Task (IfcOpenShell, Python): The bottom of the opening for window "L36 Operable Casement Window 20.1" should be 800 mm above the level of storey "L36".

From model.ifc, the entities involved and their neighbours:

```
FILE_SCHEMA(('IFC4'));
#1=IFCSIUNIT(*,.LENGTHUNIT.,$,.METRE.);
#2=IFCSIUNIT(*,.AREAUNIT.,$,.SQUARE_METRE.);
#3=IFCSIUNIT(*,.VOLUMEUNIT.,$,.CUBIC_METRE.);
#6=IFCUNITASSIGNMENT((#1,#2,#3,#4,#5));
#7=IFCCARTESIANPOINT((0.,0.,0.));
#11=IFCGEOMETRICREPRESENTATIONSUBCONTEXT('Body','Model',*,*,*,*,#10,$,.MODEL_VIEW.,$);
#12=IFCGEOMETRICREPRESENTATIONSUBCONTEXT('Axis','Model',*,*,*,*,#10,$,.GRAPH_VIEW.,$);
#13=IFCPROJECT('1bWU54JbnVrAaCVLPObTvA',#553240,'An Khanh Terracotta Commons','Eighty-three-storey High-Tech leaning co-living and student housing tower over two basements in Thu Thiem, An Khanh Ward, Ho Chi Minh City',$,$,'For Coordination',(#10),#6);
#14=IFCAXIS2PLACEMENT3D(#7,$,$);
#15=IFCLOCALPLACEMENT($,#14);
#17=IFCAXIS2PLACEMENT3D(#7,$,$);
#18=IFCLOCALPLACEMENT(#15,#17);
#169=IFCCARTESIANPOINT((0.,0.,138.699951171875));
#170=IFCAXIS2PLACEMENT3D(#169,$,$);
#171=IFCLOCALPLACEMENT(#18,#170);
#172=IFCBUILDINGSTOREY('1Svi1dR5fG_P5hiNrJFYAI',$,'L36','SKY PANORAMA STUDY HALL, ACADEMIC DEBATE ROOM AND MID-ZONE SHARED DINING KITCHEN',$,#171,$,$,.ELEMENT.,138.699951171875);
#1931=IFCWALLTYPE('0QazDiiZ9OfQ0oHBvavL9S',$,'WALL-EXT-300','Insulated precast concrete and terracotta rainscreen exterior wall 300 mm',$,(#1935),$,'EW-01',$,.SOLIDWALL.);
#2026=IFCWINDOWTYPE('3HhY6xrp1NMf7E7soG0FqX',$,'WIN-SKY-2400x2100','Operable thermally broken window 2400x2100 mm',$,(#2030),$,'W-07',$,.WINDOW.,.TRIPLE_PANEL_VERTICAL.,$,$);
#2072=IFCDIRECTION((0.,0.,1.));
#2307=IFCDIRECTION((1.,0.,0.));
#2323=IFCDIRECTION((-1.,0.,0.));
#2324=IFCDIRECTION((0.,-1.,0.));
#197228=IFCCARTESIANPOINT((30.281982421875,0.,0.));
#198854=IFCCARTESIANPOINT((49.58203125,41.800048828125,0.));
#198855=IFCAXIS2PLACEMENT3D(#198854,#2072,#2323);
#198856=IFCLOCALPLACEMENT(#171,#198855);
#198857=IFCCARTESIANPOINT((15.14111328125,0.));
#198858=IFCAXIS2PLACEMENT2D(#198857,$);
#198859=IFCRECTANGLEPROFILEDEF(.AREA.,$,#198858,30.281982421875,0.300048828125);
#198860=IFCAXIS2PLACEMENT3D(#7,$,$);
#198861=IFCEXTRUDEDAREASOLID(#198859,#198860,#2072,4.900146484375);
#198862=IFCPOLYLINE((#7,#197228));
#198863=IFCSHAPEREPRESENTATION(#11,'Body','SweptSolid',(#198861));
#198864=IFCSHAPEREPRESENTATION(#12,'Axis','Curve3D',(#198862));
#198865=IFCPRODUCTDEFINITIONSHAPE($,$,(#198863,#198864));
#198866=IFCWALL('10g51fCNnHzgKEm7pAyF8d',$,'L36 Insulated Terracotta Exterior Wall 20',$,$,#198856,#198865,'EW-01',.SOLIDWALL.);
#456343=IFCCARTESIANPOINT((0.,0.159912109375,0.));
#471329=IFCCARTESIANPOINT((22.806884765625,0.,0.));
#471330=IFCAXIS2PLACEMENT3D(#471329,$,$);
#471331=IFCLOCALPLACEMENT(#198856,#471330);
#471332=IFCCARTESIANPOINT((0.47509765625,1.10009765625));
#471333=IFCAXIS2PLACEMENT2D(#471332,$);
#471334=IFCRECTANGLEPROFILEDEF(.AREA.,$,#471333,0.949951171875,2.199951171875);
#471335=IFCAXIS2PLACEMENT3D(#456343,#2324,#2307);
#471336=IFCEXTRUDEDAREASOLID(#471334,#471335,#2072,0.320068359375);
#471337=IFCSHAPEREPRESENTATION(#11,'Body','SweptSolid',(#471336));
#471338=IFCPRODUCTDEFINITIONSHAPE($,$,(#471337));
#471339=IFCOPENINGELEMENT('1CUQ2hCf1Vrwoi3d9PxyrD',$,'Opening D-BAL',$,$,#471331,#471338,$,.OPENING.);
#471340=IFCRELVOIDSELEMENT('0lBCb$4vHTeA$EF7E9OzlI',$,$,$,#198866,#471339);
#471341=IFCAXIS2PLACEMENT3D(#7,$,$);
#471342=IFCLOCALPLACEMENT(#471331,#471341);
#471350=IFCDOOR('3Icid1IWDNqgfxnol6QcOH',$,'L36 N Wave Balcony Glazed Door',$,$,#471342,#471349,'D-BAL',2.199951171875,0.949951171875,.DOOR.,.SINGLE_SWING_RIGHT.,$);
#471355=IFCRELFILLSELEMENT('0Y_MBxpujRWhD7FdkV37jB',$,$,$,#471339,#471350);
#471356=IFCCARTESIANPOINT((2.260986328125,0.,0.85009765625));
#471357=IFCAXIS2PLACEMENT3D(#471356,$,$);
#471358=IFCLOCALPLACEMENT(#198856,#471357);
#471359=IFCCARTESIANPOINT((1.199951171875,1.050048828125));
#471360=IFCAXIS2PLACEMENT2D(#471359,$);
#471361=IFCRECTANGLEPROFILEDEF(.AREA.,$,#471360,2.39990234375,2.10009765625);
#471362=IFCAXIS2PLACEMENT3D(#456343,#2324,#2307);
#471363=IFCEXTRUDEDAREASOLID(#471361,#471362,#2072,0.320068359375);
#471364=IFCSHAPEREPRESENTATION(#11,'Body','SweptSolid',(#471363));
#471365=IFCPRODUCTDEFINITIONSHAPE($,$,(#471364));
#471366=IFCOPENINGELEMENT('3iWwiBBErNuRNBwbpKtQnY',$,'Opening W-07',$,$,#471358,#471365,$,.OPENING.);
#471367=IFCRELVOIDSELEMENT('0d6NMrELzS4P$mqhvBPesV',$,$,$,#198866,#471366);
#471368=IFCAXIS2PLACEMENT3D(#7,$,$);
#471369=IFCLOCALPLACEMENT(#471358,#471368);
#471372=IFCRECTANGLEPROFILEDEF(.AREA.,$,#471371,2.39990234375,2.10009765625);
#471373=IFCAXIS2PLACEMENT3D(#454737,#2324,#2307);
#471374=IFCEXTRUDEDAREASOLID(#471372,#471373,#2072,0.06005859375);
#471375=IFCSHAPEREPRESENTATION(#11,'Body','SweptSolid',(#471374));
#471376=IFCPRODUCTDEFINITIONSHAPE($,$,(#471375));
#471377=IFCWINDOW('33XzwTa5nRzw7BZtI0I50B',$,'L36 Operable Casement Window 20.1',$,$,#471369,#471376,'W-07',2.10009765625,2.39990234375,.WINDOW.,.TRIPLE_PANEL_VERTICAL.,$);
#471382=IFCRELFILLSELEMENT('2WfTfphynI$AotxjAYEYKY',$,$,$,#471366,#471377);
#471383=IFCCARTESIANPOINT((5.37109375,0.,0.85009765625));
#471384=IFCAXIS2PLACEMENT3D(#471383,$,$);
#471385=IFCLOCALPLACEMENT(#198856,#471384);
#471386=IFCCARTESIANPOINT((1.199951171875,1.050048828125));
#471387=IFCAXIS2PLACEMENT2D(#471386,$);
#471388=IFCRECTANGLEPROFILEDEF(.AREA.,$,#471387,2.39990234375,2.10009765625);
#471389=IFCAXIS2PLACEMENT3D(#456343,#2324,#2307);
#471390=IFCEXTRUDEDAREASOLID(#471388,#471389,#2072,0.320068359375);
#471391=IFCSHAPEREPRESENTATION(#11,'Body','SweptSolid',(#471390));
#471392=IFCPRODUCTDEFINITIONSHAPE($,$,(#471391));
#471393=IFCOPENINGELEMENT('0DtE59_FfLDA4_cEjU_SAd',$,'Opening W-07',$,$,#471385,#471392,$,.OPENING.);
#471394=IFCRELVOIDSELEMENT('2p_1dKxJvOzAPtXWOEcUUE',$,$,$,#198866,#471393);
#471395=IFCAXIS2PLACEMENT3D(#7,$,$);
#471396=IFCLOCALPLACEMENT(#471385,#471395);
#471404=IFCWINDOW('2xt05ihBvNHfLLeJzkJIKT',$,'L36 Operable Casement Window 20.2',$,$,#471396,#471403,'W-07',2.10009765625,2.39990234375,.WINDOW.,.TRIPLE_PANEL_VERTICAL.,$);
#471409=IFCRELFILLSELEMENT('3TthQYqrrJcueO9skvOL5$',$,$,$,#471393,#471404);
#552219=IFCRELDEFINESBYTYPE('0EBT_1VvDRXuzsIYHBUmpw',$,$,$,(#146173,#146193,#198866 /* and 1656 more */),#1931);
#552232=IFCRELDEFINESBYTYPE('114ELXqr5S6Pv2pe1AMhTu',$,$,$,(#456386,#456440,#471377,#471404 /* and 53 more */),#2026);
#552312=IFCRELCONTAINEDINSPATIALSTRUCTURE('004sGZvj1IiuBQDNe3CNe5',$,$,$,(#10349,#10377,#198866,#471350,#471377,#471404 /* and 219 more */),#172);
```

```python
import numpy as np
import ifcopenshell
import ifcopenshell.api.geometry
import ifcopenshell.geom
import ifcopenshell.util.element
import ifcopenshell.util.placement
import ifcopenshell.util.shape
import ifcopenshell.util.unit

model = ifcopenshell.open("model.ifc")
unit_scale = ifcopenshell.util.unit.calculate_unit_scale(model)

window = model.by_guid("33XzwTa5nRzw7BZtI0I50B")
opening = window.FillsVoids[0].RelatingOpeningElement
storey = ifcopenshell.util.element.get_container(window, ifc_class="IfcBuildingStorey")
level = ifcopenshell.util.placement.get_local_placement(storey.ObjectPlacement)[2, 3]

# The opening's origin need not be at the sill, so measure its lowest point.
shape = ifcopenshell.geom.create_shape(ifcopenshell.geom.settings(), opening)
bottom = ifcopenshell.util.shape.get_shape_bottom_elevation(shape, shape.geometry) / unit_scale
dz = level + 0.8 / unit_scale - bottom

shift = np.array([0.0, 0.0, dz])
# The window is placed relative to its opening, so it follows when the opening moves.
matrix = ifcopenshell.util.placement.get_local_placement(opening.ObjectPlacement)
matrix[:3, 3] += shift
ifcopenshell.api.geometry.edit_object_placement(
    model, product=opening, matrix=matrix, is_si=False, should_transform_children=True
)

print(f"moved by {dz * unit_scale:+.3f} m")

model.write("model_v2.ifc")
```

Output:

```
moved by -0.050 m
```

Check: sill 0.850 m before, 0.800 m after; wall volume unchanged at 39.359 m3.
